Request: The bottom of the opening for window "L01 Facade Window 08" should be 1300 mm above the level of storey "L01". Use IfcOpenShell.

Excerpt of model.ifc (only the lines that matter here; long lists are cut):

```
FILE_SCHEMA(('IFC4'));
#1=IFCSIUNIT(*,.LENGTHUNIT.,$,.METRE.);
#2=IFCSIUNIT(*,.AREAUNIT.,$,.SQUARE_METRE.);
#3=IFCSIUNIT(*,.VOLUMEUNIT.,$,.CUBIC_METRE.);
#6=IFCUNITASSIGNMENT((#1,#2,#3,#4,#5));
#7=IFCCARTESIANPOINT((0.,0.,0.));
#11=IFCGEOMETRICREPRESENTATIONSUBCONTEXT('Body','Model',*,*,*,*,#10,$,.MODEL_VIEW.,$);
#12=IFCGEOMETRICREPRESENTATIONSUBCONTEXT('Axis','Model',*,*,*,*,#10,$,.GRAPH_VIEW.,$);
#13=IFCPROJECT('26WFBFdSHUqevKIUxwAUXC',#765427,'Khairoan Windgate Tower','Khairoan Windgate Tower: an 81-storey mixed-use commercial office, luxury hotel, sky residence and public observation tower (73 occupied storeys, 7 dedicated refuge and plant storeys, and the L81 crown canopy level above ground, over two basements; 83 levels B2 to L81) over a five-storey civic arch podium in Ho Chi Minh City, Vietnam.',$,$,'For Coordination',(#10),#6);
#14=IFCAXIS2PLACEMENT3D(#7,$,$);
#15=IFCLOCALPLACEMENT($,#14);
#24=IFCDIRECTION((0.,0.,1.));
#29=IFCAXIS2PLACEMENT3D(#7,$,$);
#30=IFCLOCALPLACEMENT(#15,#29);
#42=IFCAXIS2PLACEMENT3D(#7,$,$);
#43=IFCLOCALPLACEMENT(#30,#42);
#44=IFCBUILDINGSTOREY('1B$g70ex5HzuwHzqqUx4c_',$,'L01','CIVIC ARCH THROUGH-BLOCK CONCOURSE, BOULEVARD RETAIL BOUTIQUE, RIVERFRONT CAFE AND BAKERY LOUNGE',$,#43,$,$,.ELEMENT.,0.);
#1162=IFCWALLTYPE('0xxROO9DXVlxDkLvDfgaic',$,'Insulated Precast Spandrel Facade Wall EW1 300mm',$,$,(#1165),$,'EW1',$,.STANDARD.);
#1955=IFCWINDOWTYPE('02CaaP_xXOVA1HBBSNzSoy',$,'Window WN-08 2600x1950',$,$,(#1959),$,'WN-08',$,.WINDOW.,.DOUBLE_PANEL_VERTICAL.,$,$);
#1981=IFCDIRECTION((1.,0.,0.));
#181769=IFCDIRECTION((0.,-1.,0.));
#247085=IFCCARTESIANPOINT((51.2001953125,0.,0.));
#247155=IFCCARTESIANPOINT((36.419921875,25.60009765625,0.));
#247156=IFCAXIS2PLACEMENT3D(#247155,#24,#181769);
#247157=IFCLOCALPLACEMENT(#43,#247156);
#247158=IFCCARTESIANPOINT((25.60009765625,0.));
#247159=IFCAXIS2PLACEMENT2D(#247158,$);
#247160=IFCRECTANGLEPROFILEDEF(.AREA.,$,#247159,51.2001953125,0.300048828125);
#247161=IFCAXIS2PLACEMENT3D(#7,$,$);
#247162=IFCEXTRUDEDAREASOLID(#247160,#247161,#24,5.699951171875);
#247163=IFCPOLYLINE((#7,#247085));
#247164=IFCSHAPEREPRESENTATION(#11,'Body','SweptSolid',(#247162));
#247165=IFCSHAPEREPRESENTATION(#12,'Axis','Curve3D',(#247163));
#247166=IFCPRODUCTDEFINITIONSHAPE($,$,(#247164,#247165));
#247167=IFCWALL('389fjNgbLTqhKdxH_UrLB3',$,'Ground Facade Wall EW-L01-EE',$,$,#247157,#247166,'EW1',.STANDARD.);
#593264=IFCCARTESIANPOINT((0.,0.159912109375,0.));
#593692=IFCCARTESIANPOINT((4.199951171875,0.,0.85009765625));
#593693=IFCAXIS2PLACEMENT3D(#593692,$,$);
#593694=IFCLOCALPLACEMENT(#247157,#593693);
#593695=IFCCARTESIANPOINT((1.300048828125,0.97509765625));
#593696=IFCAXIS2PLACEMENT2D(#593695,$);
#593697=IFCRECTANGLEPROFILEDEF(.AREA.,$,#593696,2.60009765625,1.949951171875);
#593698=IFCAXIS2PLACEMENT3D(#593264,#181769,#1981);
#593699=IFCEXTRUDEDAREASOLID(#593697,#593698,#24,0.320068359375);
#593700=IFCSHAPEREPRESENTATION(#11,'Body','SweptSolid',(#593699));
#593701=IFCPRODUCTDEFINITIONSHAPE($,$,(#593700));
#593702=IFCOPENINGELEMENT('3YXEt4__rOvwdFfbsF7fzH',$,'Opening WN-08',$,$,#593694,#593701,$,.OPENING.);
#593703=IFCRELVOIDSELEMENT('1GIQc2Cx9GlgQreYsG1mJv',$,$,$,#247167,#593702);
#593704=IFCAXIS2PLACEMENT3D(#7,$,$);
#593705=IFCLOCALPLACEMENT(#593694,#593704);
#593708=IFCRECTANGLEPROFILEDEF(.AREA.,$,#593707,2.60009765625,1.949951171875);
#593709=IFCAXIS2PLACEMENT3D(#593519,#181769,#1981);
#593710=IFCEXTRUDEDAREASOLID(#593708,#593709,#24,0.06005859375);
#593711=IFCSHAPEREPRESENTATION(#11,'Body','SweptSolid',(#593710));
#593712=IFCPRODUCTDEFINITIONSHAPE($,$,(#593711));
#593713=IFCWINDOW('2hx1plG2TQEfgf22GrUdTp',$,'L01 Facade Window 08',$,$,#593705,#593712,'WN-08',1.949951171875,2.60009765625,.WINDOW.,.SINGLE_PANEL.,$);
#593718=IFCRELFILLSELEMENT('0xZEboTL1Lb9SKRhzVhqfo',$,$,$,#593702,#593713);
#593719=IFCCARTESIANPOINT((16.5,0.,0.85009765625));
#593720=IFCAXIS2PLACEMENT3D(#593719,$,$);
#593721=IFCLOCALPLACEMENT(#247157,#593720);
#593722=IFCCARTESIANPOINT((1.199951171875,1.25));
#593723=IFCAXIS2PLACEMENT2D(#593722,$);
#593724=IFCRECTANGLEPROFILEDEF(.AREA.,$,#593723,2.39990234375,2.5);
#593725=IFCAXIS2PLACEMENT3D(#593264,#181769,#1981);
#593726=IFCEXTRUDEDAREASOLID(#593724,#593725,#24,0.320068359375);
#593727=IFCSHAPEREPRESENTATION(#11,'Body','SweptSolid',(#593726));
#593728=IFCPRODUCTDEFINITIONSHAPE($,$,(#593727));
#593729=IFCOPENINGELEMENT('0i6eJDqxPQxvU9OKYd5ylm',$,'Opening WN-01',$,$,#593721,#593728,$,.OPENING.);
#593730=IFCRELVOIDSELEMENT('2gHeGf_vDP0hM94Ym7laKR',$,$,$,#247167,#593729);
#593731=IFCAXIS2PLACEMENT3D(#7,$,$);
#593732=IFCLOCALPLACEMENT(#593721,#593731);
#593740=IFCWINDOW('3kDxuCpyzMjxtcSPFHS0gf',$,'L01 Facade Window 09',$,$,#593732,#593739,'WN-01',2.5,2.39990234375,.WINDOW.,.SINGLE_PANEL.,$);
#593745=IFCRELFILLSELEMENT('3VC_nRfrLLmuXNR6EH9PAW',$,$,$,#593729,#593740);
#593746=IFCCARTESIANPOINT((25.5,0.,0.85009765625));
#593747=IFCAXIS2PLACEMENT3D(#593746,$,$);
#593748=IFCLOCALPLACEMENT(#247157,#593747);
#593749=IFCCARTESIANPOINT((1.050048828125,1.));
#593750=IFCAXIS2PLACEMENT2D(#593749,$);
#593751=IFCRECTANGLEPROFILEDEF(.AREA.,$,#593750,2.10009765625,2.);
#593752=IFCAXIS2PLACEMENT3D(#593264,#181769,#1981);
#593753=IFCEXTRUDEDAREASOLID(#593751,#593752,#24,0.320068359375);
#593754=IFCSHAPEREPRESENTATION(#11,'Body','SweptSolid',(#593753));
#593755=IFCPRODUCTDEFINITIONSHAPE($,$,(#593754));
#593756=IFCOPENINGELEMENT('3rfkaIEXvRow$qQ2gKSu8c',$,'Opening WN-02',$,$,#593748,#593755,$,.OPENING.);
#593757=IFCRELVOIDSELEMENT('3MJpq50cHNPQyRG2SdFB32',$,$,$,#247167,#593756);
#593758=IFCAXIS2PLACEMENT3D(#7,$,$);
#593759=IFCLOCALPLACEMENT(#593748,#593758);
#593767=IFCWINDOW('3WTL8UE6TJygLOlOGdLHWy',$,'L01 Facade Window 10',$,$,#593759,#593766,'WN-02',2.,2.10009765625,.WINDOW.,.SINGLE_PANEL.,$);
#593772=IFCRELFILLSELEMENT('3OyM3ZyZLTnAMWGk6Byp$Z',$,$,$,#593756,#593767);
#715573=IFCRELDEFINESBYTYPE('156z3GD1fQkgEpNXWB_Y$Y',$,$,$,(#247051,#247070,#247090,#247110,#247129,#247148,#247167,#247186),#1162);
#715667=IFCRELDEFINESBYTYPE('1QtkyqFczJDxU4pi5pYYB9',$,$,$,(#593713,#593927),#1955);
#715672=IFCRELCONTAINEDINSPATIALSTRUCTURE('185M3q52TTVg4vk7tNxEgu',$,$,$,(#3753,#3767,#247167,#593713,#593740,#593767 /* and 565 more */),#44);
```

```python
import numpy as np
import ifcopenshell
import ifcopenshell.api.geometry
import ifcopenshell.geom
import ifcopenshell.util.element
import ifcopenshell.util.placement
import ifcopenshell.util.shape
import ifcopenshell.util.unit

model = ifcopenshell.open("model.ifc")
unit_scale = ifcopenshell.util.unit.calculate_unit_scale(model)

window = model.by_guid("2hx1plG2TQEfgf22GrUdTp")
opening = window.FillsVoids[0].RelatingOpeningElement
storey = ifcopenshell.util.element.get_container(window, ifc_class="IfcBuildingStorey")
level = ifcopenshell.util.placement.get_local_placement(storey.ObjectPlacement)[2, 3]

# The opening's origin need not be at the sill, so measure its lowest point.
shape = ifcopenshell.geom.create_shape(ifcopenshell.geom.settings(), opening)
bottom = ifcopenshell.util.shape.get_shape_bottom_elevation(shape, shape.geometry) / unit_scale
dz = level + 1.3 / unit_scale - bottom

shift = np.array([0.0, 0.0, dz])
# The window is placed relative to its opening, so it follows when the opening moves.
matrix = ifcopenshell.util.placement.get_local_placement(opening.ObjectPlacement)
matrix[:3, 3] += shift
ifcopenshell.api.geometry.edit_object_placement(
    model, product=opening, matrix=matrix, is_si=False, should_transform_children=True
)

print(f"moved by {dz * unit_scale:+.3f} m")

model.write("model_edited.ifc")
```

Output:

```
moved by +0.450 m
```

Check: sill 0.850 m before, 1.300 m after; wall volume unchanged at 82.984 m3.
